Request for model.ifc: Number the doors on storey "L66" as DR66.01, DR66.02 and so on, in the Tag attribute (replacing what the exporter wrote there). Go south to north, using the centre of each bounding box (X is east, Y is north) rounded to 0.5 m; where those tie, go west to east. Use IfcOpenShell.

First a look at what the model holds.

```python
import ifcopenshell
import ifcopenshell.util.element
import ifcopenshell.util.placement

model = ifcopenshell.open("model.ifc")
print(model.schema)
storey = next(s for s in model.by_type("IfcBuildingStorey") if s.Name == "L66")
doors = [e for e in ifcopenshell.util.element.get_decomposition(storey) if e.is_a("IfcDoor")]
for e in sorted(doors, key=lambda e: e.id()):
    origin = ifcopenshell.util.placement.get_local_placement(e.ObjectPlacement)[:3, 3]
    print(e.id(), e.Tag, e.Name, origin.round(2) + 0.0, sep=" | ")
```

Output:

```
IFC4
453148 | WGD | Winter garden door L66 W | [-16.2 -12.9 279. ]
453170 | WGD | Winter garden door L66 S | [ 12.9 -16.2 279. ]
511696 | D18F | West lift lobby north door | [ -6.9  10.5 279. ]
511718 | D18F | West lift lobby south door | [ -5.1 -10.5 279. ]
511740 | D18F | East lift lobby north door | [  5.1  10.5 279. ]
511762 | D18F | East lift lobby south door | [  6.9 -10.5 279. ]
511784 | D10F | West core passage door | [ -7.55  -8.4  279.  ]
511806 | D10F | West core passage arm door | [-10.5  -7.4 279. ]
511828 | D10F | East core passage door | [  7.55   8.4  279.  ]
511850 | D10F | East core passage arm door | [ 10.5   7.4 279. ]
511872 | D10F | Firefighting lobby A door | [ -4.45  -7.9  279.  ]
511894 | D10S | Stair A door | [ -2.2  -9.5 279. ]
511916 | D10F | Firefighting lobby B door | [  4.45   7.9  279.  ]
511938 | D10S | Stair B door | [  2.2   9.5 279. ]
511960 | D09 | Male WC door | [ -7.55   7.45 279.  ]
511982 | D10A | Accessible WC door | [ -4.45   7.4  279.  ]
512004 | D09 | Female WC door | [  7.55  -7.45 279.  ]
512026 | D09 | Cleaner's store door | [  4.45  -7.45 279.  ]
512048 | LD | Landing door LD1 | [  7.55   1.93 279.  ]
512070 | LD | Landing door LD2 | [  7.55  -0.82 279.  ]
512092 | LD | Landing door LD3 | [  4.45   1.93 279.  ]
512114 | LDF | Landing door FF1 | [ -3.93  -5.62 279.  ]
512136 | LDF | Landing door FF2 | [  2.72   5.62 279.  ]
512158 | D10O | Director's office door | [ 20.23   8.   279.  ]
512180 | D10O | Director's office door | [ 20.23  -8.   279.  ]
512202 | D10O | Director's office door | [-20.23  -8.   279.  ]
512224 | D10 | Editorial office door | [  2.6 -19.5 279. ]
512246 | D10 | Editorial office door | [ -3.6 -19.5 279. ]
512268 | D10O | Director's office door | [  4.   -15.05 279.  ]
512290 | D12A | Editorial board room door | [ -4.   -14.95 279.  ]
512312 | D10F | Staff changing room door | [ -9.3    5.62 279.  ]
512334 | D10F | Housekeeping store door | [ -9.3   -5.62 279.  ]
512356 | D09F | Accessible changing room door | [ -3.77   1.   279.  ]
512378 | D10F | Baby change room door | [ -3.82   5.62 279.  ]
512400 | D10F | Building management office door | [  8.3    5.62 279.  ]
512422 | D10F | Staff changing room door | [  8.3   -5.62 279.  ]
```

```python
import ifcopenshell
import ifcopenshell.geom
import ifcopenshell.util.element
import ifcopenshell.util.shape

model = ifcopenshell.open("model.ifc")
settings = ifcopenshell.geom.settings()
settings.set("use-world-coords", True)


def centre(element):
    shape = ifcopenshell.geom.create_shape(settings, element)
    return ifcopenshell.util.shape.get_bbox_centroid(shape.geometry)


storey = next(s for s in model.by_type("IfcBuildingStorey") if s.Name == "L66")
doors = [e for e in ifcopenshell.util.element.get_decomposition(storey) if e.is_a("IfcDoor")]

# Insertion points can sit at a corner or the storey origin, so sort by the geometry (in metres).
centres = {e: centre(e) for e in doors}
doors.sort(key=lambda e: (round(centres[e][1] / 0.5), centres[e][0]))

for i, e in enumerate(doors, start=1):
    number = f"DR66.{i:02d}"
    e.Tag = number
    print(e.id(), number)

model.write("model_edited.ifc")
```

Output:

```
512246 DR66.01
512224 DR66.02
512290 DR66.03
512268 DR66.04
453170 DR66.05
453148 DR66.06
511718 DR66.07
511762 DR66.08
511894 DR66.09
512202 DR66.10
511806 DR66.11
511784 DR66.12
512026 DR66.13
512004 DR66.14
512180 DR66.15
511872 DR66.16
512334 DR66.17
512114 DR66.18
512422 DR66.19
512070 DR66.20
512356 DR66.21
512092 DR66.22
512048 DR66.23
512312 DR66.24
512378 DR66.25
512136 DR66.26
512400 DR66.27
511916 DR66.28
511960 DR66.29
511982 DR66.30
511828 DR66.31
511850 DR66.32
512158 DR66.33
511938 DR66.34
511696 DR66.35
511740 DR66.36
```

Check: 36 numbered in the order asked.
